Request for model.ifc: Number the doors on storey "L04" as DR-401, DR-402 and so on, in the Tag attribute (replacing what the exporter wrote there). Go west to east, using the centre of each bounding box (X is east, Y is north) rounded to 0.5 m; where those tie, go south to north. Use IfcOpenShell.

First a look at what the model holds.

```python
import ifcopenshell
import ifcopenshell.util.element
import ifcopenshell.util.placement

model = ifcopenshell.open("model.ifc")
print(model.schema)
storey = next(s for s in model.by_type("IfcBuildingStorey") if s.Name == "L04")
doors = [e for e in ifcopenshell.util.element.get_decomposition(storey) if e.is_a("IfcDoor")]
for e in sorted(doors, key=lambda e: e.id()):
    origin = ifcopenshell.util.placement.get_local_placement(e.ObjectPlacement)[:3, 3]
    print(e.id(), e.Tag, e.Name, origin.round(2) + 0.0, sep=" | ")
```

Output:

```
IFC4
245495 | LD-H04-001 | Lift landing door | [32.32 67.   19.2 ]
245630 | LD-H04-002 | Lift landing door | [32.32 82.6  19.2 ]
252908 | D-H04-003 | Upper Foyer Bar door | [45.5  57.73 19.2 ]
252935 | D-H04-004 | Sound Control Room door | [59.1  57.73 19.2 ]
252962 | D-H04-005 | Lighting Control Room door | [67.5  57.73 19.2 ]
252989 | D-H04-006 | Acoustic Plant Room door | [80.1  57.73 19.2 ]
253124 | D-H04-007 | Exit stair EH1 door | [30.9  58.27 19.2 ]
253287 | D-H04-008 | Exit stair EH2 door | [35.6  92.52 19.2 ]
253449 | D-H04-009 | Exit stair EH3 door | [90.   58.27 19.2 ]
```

```python
import ifcopenshell
import ifcopenshell.geom
import ifcopenshell.util.element
import ifcopenshell.util.shape

model = ifcopenshell.open("model.ifc")
settings = ifcopenshell.geom.settings()
settings.set("use-world-coords", True)


def centre(element):
    shape = ifcopenshell.geom.create_shape(settings, element)
    return ifcopenshell.util.shape.get_bbox_centroid(shape.geometry)


storey = next(s for s in model.by_type("IfcBuildingStorey") if s.Name == "L04")
doors = [e for e in ifcopenshell.util.element.get_decomposition(storey) if e.is_a("IfcDoor")]

# Insertion points can sit at a corner or the storey origin, so sort by the geometry (in metres).
centres = {e: centre(e) for e in doors}
doors.sort(key=lambda e: (round(centres[e][0] / 0.5), centres[e][1]))

for i, e in enumerate(doors, start=1):
    number = f"DR-4{i:02d}"
    e.Tag = number
    print(e.id(), number)

model.write("model_updated.ifc")
```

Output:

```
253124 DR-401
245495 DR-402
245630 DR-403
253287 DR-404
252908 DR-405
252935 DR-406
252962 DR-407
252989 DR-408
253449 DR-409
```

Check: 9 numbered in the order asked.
